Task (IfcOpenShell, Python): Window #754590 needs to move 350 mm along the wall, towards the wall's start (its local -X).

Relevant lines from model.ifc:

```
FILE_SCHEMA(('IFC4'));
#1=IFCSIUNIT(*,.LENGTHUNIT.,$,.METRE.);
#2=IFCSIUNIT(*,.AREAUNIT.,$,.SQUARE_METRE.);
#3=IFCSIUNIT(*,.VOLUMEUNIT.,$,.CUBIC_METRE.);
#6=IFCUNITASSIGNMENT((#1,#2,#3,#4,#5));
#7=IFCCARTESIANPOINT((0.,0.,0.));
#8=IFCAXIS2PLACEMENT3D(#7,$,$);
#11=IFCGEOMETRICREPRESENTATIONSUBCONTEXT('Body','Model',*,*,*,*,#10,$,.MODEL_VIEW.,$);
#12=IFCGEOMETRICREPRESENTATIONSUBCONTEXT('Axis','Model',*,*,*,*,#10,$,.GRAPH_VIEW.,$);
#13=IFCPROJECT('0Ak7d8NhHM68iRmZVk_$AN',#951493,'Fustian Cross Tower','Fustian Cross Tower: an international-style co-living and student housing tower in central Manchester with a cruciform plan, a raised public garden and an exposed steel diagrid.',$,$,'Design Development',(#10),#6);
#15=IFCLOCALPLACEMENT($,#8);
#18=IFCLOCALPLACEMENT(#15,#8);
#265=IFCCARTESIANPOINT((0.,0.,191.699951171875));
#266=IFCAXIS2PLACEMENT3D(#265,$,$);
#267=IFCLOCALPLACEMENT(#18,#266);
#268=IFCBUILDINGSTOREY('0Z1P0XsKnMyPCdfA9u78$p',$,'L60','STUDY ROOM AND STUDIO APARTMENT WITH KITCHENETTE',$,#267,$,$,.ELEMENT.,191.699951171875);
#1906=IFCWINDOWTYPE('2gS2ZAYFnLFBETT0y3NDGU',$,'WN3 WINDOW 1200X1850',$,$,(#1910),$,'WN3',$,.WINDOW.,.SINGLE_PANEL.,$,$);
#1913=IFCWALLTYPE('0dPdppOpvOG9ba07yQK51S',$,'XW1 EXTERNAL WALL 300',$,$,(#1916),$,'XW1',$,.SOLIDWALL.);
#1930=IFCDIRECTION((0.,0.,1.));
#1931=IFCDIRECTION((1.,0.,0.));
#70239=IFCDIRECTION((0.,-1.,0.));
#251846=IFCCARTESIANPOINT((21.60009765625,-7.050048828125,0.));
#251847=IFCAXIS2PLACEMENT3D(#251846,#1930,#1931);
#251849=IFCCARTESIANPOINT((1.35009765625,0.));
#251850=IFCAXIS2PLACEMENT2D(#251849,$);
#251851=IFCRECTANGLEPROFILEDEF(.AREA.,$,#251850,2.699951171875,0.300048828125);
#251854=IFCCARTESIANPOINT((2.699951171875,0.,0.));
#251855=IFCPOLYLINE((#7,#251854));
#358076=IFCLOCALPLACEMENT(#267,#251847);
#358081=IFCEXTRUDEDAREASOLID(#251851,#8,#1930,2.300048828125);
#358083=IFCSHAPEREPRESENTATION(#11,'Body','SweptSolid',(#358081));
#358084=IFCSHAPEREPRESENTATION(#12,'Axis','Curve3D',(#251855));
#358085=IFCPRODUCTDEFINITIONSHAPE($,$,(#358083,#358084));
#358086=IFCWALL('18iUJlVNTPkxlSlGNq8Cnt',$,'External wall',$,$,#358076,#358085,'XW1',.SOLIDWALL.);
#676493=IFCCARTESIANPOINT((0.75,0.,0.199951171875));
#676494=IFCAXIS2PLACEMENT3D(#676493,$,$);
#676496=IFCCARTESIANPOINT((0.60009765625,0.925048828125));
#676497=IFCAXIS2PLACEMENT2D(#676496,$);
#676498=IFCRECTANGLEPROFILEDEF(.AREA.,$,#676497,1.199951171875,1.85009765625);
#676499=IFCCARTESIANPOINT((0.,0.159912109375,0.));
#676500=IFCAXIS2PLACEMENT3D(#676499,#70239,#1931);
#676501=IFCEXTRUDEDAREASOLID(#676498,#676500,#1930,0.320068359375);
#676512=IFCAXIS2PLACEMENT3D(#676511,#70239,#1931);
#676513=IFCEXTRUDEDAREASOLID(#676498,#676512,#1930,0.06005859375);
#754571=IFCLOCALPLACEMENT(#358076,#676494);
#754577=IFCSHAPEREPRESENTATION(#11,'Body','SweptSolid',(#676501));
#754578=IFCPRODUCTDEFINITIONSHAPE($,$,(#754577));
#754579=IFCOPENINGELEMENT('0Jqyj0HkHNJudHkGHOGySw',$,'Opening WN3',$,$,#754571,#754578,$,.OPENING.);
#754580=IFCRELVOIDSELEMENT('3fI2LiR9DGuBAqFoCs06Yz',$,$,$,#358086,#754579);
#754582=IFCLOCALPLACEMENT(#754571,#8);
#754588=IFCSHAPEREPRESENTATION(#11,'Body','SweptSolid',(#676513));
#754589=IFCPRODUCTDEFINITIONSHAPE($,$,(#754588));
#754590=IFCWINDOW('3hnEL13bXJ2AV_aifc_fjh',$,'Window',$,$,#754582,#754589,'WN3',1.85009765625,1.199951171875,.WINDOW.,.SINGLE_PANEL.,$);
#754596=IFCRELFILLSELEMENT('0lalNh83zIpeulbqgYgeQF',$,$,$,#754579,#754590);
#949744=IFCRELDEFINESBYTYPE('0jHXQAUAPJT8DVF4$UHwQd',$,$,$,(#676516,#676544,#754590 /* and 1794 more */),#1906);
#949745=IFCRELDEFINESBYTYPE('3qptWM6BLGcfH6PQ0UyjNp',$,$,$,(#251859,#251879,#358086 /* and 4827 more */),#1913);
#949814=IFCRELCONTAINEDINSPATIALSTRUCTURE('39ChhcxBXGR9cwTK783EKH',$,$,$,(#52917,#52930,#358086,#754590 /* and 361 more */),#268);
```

```python
import ifcopenshell
import ifcopenshell.api.geometry
import ifcopenshell.util.placement
import ifcopenshell.util.unit

model = ifcopenshell.open("model.ifc")
unit_scale = ifcopenshell.util.unit.calculate_unit_scale(model)

window = model.by_guid("3hnEL13bXJ2AV_aifc_fjh")
opening = window.FillsVoids[0].RelatingOpeningElement
wall = opening.VoidsElements[0].RelatingBuildingElement

wall_matrix = ifcopenshell.util.placement.get_local_placement(wall.ObjectPlacement)
shift = wall_matrix[:3, 0] * -0.35 / unit_scale
before = ifcopenshell.util.placement.get_local_placement(window.ObjectPlacement)[:3, 3].copy()

# The window is placed relative to its opening, so it follows when the opening moves.
matrix = ifcopenshell.util.placement.get_local_placement(opening.ObjectPlacement)
matrix[:3, 3] += shift
ifcopenshell.api.geometry.edit_object_placement(
    model, product=opening, matrix=matrix, is_si=False, should_transform_children=True
)

after = ifcopenshell.util.placement.get_local_placement(window.ObjectPlacement)[:3, 3]
print("window moved by", (after - before).round(3) + 0.0)

model.write("model_rev.ifc")
```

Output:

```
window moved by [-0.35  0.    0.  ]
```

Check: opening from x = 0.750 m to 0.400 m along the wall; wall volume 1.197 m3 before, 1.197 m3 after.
